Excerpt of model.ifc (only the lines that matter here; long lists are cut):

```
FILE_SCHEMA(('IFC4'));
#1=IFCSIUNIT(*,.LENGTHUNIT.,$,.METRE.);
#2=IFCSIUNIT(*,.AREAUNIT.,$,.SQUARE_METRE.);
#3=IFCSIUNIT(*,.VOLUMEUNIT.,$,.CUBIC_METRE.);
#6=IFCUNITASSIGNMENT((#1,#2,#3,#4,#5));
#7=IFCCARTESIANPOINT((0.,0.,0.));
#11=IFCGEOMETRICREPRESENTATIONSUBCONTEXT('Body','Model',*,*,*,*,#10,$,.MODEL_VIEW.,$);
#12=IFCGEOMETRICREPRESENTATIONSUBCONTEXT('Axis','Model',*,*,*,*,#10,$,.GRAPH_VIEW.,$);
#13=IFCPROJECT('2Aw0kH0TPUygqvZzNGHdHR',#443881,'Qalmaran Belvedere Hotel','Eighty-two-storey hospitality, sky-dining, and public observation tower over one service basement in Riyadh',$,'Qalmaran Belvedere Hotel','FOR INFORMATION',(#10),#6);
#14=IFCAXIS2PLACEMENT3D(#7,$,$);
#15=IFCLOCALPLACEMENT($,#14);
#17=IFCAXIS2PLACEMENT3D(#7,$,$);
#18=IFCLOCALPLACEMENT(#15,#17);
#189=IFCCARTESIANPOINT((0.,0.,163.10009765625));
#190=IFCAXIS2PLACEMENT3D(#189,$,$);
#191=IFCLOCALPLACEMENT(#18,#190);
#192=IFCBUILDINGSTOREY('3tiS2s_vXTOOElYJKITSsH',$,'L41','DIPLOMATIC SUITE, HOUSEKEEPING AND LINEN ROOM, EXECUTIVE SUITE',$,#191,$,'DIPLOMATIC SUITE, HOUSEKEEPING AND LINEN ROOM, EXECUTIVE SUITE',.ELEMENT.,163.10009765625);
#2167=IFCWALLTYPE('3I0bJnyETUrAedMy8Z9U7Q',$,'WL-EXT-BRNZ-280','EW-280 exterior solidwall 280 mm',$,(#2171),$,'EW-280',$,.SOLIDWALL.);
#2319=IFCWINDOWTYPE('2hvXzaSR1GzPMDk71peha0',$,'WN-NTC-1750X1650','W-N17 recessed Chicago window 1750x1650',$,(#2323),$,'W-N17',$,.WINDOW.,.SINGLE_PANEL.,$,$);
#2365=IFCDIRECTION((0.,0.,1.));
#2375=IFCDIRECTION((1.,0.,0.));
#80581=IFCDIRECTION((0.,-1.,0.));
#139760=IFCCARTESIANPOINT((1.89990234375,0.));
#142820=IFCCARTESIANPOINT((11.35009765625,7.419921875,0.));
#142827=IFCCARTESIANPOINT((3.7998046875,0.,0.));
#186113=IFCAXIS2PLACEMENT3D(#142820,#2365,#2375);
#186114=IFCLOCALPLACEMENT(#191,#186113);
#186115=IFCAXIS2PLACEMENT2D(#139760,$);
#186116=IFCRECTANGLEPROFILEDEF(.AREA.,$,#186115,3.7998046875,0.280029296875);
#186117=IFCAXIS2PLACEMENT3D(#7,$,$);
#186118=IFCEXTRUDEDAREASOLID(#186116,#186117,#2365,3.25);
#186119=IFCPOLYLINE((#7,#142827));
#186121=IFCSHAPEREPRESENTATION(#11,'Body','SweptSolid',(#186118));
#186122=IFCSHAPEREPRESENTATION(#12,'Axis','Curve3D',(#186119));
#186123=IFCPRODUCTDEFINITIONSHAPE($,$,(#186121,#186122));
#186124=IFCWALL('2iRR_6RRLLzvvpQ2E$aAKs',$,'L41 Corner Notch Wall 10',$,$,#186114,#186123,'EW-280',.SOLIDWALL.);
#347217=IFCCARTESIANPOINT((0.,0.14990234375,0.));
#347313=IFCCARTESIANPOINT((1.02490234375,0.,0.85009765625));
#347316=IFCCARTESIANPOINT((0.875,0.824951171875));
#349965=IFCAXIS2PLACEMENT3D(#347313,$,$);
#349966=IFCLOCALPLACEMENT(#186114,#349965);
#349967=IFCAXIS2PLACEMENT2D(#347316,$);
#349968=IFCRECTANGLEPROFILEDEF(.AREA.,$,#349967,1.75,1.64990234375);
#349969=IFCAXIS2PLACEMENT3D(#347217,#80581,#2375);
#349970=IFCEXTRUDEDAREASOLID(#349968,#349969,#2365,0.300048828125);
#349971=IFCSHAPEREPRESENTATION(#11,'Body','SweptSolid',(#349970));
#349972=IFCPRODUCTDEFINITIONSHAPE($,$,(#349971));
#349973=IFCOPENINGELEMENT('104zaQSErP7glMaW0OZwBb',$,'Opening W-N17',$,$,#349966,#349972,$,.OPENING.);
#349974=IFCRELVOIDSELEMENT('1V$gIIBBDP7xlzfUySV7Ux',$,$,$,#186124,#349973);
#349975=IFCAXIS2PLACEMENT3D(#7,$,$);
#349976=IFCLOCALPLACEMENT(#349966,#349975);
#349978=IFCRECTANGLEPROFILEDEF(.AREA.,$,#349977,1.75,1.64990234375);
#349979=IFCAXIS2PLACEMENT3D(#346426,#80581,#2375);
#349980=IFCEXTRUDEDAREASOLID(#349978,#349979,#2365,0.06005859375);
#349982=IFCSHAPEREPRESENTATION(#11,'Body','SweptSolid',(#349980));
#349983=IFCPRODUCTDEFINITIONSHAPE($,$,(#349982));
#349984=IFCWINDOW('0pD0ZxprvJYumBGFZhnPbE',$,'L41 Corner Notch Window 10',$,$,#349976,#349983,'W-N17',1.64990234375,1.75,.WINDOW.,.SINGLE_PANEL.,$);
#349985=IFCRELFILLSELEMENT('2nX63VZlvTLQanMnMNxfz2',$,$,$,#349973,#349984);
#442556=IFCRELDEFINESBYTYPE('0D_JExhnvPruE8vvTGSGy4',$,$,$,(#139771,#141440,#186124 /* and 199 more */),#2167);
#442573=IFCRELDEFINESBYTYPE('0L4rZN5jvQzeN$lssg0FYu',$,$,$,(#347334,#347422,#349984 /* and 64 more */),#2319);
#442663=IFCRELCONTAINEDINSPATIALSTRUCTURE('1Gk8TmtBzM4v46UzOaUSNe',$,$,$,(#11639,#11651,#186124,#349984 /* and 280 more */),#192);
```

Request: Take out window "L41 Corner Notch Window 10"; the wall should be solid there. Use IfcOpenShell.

```python
import ifcopenshell
import ifcopenshell.api.feature
import ifcopenshell.api.root
import ifcopenshell.geom
import ifcopenshell.util.shape

model = ifcopenshell.open("model.ifc")
settings = ifcopenshell.geom.settings()


def volume(element):
    """Net volume in cubic metres, openings subtracted."""
    shape = ifcopenshell.geom.create_shape(settings, element)
    return ifcopenshell.util.shape.get_volume(shape.geometry)


window = model.by_guid("0pD0ZxprvJYumBGFZhnPbE")
opening = window.FillsVoids[0].RelatingOpeningElement
wall = opening.VoidsElements[0].RelatingBuildingElement
before = volume(wall)

ifcopenshell.api.root.remove_product(model, product=window)
ifcopenshell.api.feature.remove_feature(model, feature=opening)

after = volume(wall)

print(f"wall volume {before:.3f} -> {after:.3f} m3")

model.write("model_edited.ifc")
```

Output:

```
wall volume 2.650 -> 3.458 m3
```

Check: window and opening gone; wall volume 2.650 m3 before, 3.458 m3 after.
